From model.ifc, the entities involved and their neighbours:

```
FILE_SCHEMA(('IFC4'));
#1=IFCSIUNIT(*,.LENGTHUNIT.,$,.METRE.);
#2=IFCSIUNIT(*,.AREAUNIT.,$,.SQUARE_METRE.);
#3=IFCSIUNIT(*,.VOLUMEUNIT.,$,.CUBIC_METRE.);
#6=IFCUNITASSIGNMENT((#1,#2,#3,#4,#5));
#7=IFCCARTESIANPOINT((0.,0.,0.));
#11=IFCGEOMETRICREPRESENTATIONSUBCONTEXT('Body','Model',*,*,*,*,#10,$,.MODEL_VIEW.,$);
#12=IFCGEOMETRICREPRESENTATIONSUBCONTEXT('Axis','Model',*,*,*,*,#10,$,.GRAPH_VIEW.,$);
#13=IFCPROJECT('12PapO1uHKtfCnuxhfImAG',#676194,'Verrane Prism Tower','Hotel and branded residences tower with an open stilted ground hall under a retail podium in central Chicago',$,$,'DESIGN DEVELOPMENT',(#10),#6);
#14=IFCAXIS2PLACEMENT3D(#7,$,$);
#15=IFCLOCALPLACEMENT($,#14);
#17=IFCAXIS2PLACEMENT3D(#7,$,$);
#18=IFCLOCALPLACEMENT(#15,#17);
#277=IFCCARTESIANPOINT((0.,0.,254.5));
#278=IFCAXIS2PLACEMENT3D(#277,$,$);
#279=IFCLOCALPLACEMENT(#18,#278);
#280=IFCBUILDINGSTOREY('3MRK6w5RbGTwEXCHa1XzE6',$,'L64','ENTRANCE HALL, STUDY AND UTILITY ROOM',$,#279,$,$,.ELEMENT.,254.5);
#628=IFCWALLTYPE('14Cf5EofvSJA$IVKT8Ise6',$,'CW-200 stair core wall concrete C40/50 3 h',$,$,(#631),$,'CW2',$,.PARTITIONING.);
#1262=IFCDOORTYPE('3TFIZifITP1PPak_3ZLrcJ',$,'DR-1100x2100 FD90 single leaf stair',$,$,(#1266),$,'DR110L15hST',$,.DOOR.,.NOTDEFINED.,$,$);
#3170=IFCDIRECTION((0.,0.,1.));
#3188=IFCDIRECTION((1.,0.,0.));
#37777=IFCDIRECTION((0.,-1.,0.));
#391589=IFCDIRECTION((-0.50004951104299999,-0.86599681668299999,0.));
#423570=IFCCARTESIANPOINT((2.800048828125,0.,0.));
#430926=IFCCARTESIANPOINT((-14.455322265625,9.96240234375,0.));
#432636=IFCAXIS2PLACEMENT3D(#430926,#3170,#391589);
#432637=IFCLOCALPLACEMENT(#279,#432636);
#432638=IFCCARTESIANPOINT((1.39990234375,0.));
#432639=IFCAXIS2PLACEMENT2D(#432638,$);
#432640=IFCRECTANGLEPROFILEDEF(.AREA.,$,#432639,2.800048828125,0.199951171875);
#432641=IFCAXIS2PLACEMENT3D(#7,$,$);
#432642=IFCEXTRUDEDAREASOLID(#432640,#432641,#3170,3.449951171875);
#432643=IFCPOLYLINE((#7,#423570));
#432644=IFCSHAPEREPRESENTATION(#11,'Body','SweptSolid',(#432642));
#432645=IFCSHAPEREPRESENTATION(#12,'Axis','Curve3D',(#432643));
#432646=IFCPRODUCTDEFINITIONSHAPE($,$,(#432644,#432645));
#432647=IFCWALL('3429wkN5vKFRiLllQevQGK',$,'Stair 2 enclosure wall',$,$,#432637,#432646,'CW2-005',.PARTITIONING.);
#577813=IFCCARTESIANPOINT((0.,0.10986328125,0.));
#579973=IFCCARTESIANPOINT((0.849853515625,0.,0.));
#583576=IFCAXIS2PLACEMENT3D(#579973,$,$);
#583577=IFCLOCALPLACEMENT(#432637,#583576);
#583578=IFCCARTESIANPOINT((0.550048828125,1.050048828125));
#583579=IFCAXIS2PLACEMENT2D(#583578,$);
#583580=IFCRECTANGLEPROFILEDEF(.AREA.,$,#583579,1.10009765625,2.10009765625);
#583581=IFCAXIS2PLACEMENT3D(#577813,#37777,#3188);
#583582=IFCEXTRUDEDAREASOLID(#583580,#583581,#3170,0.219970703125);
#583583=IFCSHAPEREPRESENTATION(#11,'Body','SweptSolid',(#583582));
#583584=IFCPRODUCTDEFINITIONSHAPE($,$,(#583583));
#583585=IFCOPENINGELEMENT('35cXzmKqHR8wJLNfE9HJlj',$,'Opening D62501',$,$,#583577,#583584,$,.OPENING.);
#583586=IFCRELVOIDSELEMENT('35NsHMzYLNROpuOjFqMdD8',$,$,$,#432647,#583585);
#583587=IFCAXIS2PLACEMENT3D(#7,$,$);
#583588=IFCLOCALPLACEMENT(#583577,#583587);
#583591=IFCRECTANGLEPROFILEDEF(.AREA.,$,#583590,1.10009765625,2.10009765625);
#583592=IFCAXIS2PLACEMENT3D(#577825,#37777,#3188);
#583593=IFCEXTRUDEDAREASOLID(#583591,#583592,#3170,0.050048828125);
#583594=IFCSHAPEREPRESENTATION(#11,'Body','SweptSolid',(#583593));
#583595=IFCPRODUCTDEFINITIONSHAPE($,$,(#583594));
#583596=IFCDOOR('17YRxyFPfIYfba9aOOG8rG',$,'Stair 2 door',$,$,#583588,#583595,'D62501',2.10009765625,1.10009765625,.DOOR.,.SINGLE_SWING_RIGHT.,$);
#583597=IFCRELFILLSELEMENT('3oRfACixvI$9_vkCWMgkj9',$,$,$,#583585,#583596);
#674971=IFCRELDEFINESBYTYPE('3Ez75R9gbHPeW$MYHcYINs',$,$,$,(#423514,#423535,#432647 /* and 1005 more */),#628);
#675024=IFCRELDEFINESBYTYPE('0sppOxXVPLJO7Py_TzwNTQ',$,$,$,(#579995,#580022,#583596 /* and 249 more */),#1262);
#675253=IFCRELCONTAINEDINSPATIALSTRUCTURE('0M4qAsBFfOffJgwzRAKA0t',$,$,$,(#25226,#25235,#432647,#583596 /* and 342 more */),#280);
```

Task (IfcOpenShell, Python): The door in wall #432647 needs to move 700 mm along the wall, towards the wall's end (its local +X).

```python
import ifcopenshell
import ifcopenshell.api.geometry
import ifcopenshell.util.placement
import ifcopenshell.util.unit

model = ifcopenshell.open("model.ifc")
unit_scale = ifcopenshell.util.unit.calculate_unit_scale(model)

door = model.by_guid("17YRxyFPfIYfba9aOOG8rG")
opening = door.FillsVoids[0].RelatingOpeningElement
wall = opening.VoidsElements[0].RelatingBuildingElement

wall_matrix = ifcopenshell.util.placement.get_local_placement(wall.ObjectPlacement)
shift = wall_matrix[:3, 0] * 0.7 / unit_scale
before = ifcopenshell.util.placement.get_local_placement(door.ObjectPlacement)[:3, 3].copy()

# The door is placed relative to its opening, so it follows when the opening moves.
matrix = ifcopenshell.util.placement.get_local_placement(opening.ObjectPlacement)
matrix[:3, 3] += shift
ifcopenshell.api.geometry.edit_object_placement(
    model, product=opening, matrix=matrix, is_si=False, should_transform_children=True
)

after = ifcopenshell.util.placement.get_local_placement(door.ObjectPlacement)[:3, 3]
print("door moved by", (after - before).round(3) + 0.0)

model.write("model_rev.ifc")
```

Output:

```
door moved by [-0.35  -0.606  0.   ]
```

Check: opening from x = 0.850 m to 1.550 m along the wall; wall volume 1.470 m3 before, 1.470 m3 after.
